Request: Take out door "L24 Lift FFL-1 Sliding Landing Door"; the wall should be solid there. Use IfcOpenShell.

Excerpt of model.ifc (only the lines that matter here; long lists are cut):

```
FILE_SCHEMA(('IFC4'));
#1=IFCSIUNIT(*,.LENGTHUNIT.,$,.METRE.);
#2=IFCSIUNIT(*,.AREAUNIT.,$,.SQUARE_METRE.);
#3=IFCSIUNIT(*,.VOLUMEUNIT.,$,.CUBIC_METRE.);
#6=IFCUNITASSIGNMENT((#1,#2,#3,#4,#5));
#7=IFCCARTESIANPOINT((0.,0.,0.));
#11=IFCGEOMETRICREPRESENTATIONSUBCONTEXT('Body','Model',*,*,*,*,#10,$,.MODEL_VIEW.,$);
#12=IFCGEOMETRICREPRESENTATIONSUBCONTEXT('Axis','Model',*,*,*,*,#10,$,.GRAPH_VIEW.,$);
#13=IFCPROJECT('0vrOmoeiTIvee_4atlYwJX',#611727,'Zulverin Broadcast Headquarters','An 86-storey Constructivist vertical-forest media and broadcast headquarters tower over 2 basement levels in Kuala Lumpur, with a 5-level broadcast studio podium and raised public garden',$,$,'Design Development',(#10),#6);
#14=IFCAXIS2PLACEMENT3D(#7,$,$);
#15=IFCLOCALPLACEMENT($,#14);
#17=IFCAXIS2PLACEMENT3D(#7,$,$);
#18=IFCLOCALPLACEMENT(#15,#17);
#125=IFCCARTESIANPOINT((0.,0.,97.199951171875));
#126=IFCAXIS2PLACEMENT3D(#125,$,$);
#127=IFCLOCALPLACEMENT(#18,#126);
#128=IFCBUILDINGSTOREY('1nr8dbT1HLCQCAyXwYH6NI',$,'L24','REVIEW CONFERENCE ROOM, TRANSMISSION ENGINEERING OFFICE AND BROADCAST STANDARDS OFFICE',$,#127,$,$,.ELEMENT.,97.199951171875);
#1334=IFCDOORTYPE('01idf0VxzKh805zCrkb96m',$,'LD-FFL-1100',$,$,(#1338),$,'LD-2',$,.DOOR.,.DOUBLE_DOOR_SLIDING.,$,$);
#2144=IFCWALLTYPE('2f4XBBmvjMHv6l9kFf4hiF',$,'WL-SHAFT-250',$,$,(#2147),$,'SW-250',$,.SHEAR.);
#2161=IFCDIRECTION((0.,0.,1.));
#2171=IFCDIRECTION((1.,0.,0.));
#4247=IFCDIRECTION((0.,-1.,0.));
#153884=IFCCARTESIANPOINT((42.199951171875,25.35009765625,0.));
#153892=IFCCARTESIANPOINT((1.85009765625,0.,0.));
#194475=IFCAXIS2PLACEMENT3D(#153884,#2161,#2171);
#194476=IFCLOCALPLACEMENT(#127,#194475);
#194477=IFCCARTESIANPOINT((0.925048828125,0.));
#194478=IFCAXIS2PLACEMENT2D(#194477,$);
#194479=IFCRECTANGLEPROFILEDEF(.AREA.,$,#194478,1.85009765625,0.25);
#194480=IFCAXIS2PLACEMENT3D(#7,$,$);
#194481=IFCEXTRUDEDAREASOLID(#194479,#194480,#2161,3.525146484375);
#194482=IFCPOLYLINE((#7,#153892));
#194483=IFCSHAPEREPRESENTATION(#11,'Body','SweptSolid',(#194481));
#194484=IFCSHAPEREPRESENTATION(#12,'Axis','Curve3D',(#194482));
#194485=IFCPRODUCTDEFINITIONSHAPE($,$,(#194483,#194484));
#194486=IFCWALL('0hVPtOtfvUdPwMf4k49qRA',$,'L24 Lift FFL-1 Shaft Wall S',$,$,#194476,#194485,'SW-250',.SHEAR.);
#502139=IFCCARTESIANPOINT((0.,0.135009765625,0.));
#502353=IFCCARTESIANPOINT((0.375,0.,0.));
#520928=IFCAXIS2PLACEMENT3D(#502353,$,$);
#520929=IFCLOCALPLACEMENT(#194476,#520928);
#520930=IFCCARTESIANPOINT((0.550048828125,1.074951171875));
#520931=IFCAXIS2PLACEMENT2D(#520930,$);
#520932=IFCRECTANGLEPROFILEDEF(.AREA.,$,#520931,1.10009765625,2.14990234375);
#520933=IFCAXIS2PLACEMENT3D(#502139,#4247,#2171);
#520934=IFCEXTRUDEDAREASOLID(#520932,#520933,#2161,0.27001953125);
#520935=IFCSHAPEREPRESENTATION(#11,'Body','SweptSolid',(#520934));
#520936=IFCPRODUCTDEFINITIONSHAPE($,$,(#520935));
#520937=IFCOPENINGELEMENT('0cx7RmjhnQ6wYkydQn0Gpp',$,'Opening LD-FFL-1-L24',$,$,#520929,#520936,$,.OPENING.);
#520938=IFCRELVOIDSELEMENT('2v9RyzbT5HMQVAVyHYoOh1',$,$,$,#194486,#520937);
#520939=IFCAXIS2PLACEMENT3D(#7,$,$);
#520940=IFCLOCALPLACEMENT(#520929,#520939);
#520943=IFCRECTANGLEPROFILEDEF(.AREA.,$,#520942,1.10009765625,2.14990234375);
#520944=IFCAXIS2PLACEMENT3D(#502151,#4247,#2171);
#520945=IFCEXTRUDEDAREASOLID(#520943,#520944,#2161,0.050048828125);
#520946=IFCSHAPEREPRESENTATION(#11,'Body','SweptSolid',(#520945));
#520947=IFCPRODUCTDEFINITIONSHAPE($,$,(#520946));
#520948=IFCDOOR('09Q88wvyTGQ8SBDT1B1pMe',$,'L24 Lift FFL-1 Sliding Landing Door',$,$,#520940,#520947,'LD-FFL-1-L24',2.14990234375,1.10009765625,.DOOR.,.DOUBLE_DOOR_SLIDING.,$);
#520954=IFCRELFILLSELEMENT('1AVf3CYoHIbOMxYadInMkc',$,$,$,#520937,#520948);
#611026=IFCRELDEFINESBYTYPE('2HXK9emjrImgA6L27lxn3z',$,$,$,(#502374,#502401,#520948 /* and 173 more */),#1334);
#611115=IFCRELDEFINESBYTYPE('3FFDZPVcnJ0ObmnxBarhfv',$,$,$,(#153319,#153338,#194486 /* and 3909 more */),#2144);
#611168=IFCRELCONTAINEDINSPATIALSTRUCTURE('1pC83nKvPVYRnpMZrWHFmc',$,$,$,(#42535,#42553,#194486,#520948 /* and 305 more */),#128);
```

```python
import ifcopenshell
import ifcopenshell.api.feature
import ifcopenshell.api.root
import ifcopenshell.geom
import ifcopenshell.util.shape

model = ifcopenshell.open("model.ifc")
settings = ifcopenshell.geom.settings()


def volume(element):
    """Net volume in cubic metres, openings subtracted."""
    shape = ifcopenshell.geom.create_shape(settings, element)
    return ifcopenshell.util.shape.get_volume(shape.geometry)


door = model.by_guid("09Q88wvyTGQ8SBDT1B1pMe")
opening = door.FillsVoids[0].RelatingOpeningElement
wall = opening.VoidsElements[0].RelatingBuildingElement
before = volume(wall)

ifcopenshell.api.root.remove_product(model, product=door)
ifcopenshell.api.feature.remove_feature(model, feature=opening)

after = volume(wall)

print(f"wall volume {before:.3f} -> {after:.3f} m3")

model.write("model-out.ifc")
```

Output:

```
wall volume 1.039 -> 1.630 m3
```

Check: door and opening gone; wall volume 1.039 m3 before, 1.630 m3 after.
